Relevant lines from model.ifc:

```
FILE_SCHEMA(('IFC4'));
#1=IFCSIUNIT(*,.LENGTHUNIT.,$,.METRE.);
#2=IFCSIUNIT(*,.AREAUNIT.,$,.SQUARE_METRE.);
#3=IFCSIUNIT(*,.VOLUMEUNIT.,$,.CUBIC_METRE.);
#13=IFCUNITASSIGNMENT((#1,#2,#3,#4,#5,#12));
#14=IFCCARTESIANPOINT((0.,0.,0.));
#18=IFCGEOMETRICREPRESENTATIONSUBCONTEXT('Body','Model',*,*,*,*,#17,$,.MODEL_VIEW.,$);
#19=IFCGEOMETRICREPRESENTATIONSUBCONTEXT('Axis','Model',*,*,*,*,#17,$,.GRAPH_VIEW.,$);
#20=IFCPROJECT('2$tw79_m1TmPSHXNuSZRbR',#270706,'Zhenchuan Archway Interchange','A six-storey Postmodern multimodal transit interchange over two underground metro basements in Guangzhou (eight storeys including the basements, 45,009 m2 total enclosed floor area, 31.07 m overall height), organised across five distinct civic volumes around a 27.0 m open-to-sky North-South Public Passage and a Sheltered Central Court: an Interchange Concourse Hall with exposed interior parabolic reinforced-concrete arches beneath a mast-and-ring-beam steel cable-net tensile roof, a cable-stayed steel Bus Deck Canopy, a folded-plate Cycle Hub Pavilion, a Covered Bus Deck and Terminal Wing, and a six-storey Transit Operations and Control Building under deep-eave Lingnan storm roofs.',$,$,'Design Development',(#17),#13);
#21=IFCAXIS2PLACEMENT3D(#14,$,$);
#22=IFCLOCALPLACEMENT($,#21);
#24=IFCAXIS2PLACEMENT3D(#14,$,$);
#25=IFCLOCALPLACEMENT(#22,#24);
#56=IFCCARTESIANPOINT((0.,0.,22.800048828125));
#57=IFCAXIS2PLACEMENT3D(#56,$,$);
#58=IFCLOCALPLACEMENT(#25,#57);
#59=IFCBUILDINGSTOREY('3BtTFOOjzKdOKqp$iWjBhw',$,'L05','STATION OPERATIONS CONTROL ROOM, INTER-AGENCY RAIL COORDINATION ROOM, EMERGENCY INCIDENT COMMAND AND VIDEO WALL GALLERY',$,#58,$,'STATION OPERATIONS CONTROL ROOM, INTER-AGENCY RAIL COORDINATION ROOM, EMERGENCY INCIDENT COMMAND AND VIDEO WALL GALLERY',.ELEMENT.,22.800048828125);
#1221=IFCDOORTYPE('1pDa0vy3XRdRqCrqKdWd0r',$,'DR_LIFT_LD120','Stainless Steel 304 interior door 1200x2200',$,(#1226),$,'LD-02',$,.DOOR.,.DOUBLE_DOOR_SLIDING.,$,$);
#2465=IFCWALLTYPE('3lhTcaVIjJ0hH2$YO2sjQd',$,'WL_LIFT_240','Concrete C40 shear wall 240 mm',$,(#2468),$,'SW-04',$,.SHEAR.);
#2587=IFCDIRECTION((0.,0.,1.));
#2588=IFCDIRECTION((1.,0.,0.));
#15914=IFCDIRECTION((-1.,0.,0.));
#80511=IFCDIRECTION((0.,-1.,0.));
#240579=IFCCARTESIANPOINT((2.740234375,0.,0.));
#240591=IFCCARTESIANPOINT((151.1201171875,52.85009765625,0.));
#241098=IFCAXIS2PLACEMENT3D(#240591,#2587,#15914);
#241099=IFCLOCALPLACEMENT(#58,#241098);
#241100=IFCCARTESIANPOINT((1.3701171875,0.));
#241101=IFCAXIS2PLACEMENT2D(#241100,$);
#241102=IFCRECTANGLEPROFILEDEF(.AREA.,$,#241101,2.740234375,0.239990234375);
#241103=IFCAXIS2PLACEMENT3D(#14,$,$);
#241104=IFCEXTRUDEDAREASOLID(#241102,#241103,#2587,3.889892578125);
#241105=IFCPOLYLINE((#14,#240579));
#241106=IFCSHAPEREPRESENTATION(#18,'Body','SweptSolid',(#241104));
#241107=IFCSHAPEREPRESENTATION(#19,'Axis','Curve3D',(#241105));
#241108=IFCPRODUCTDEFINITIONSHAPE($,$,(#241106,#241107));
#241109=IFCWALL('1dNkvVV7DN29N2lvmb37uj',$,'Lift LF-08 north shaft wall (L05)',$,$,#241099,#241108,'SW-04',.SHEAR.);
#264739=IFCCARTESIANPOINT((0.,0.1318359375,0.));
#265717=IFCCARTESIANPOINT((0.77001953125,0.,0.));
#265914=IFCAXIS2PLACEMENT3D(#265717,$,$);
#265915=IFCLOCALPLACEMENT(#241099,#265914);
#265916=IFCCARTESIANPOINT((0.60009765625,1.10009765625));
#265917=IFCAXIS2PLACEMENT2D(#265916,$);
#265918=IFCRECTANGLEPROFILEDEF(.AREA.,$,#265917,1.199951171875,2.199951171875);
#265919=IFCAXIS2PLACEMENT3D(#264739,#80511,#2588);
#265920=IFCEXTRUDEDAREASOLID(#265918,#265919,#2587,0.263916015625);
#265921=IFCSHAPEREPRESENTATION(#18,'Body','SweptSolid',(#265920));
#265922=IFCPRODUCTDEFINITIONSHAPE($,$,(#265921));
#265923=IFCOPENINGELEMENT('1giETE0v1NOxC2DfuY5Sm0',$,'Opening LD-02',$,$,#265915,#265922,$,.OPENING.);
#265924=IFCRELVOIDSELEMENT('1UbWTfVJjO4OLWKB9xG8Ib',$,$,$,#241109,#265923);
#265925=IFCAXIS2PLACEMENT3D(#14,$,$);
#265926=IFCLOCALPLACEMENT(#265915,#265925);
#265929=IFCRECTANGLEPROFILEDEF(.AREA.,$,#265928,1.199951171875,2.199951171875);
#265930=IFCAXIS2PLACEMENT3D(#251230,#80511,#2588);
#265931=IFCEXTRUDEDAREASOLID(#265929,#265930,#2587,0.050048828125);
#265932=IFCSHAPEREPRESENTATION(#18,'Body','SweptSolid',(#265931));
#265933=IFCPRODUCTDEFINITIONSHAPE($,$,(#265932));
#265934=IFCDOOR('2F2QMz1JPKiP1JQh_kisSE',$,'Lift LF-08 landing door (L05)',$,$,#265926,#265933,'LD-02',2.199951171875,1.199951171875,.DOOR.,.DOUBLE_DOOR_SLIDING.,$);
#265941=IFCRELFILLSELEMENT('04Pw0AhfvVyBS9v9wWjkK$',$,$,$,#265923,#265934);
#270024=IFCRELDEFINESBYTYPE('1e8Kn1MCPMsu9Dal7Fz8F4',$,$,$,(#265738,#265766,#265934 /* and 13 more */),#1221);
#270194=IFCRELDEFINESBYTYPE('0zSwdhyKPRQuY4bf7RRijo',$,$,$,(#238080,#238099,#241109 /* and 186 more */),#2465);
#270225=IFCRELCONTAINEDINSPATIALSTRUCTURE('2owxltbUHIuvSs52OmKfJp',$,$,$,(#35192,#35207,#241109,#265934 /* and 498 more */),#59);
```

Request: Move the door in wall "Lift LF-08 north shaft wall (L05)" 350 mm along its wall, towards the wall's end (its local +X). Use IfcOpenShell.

```python
import ifcopenshell
import ifcopenshell.api.geometry
import ifcopenshell.util.placement

model = ifcopenshell.open("model.ifc")

door = model.by_guid("2F2QMz1JPKiP1JQh_kisSE")
opening = door.FillsVoids[0].RelatingOpeningElement
wall = opening.VoidsElements[0].RelatingBuildingElement

wall_matrix = ifcopenshell.util.placement.get_local_placement(wall.ObjectPlacement)
shift = wall_matrix[:3, 0] * 0.35
before = ifcopenshell.util.placement.get_local_placement(door.ObjectPlacement)[:3, 3].copy()

# The door is placed relative to its opening, so it follows when the opening moves.
matrix = ifcopenshell.util.placement.get_local_placement(opening.ObjectPlacement)
matrix[:3, 3] += shift
ifcopenshell.api.geometry.edit_object_placement(
    model, product=opening, matrix=matrix, is_si=False, should_transform_children=True
)

after = ifcopenshell.util.placement.get_local_placement(door.ObjectPlacement)[:3, 3]
print("door moved by", (after - before).round(3) + 0.0)

model.write("model_edited.ifc")
```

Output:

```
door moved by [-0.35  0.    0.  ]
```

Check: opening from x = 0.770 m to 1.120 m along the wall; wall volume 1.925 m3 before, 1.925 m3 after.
